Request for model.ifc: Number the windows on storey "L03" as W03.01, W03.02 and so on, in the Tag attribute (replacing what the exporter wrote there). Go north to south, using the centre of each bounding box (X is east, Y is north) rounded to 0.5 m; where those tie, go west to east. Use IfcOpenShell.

First a look at what the model holds.

```python
import ifcopenshell
import ifcopenshell.util.element
import ifcopenshell.util.placement

model = ifcopenshell.open("model.ifc")
print(model.schema)
storey = next(s for s in model.by_type("IfcBuildingStorey") if s.Name == "L03")
windows = [e for e in ifcopenshell.util.element.get_decomposition(storey) if e.is_a("IfcWindow")]
for e in sorted(windows, key=lambda e: e.id()):
    origin = ifcopenshell.util.placement.get_local_placement(e.ObjectPlacement)[:3, 3]
    print(e.id(), e.Tag, e.Name, origin.round(2) + 0.0, sep=" | ")
```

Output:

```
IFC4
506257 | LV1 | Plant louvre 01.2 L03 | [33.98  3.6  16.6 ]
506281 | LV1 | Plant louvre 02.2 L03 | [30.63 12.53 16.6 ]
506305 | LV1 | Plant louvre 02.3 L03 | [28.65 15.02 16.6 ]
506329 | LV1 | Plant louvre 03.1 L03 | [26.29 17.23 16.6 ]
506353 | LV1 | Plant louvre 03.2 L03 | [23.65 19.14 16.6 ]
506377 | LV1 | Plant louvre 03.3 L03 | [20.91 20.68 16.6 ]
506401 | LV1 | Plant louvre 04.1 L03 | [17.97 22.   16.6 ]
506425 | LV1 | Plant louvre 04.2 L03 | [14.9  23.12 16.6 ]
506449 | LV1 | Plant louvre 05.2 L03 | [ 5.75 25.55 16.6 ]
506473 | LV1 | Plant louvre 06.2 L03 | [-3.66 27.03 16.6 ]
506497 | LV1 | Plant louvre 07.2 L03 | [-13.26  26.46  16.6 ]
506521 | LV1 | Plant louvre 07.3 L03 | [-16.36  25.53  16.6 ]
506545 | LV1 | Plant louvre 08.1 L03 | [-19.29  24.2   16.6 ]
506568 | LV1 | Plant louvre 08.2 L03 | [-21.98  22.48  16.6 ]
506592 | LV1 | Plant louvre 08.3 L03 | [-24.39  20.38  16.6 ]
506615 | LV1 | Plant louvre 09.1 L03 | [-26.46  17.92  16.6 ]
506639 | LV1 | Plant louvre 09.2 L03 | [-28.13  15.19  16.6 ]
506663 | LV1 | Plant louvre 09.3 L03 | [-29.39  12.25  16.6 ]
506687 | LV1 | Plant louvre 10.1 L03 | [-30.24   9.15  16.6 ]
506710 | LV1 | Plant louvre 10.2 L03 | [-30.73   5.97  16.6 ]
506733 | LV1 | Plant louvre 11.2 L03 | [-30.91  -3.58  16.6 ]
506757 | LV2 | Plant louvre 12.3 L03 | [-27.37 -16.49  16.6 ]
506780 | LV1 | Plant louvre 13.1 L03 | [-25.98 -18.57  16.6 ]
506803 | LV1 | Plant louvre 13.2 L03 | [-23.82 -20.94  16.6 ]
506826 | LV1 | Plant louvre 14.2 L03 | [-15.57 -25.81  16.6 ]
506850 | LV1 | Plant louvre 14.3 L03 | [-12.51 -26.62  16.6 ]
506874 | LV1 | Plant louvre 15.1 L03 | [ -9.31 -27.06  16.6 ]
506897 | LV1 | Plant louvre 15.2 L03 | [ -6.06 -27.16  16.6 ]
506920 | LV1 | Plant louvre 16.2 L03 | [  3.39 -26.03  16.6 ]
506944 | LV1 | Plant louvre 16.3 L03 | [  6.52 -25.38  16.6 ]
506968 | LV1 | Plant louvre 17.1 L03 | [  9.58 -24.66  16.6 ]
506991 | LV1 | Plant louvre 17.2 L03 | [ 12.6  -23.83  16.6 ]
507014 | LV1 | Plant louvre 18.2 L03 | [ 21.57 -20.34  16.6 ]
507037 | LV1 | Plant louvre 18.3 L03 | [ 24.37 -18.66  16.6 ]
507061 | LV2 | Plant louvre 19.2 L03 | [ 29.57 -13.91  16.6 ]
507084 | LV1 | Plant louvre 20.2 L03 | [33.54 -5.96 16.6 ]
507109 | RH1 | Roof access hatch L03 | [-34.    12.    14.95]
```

```python
import ifcopenshell
import ifcopenshell.geom
import ifcopenshell.util.element
import ifcopenshell.util.shape

model = ifcopenshell.open("model.ifc")
settings = ifcopenshell.geom.settings()
settings.set("use-world-coords", True)


def centre(element):
    shape = ifcopenshell.geom.create_shape(settings, element)
    return ifcopenshell.util.shape.get_bbox_centroid(shape.geometry)


storey = next(s for s in model.by_type("IfcBuildingStorey") if s.Name == "L03")
windows = [e for e in ifcopenshell.util.element.get_decomposition(storey) if e.is_a("IfcWindow")]

# Insertion points can sit at a corner or the storey origin, so sort by the geometry (in metres).
centres = {e: centre(e) for e in windows}
windows.sort(key=lambda e: (-round(centres[e][1] / 0.5), centres[e][0]))

for i, e in enumerate(windows, start=1):
    number = f"W03.{i:02d}"
    e.Tag = number
    print(e.id(), number)

model.write("model_updated.ifc")
```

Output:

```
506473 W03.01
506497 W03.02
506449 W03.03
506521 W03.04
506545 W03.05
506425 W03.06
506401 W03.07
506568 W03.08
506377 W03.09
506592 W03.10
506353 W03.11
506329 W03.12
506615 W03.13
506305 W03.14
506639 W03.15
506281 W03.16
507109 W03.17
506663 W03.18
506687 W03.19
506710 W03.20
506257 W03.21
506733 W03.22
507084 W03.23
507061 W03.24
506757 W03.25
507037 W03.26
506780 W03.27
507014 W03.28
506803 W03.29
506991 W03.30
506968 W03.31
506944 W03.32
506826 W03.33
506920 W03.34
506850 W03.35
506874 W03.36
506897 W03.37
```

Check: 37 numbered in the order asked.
